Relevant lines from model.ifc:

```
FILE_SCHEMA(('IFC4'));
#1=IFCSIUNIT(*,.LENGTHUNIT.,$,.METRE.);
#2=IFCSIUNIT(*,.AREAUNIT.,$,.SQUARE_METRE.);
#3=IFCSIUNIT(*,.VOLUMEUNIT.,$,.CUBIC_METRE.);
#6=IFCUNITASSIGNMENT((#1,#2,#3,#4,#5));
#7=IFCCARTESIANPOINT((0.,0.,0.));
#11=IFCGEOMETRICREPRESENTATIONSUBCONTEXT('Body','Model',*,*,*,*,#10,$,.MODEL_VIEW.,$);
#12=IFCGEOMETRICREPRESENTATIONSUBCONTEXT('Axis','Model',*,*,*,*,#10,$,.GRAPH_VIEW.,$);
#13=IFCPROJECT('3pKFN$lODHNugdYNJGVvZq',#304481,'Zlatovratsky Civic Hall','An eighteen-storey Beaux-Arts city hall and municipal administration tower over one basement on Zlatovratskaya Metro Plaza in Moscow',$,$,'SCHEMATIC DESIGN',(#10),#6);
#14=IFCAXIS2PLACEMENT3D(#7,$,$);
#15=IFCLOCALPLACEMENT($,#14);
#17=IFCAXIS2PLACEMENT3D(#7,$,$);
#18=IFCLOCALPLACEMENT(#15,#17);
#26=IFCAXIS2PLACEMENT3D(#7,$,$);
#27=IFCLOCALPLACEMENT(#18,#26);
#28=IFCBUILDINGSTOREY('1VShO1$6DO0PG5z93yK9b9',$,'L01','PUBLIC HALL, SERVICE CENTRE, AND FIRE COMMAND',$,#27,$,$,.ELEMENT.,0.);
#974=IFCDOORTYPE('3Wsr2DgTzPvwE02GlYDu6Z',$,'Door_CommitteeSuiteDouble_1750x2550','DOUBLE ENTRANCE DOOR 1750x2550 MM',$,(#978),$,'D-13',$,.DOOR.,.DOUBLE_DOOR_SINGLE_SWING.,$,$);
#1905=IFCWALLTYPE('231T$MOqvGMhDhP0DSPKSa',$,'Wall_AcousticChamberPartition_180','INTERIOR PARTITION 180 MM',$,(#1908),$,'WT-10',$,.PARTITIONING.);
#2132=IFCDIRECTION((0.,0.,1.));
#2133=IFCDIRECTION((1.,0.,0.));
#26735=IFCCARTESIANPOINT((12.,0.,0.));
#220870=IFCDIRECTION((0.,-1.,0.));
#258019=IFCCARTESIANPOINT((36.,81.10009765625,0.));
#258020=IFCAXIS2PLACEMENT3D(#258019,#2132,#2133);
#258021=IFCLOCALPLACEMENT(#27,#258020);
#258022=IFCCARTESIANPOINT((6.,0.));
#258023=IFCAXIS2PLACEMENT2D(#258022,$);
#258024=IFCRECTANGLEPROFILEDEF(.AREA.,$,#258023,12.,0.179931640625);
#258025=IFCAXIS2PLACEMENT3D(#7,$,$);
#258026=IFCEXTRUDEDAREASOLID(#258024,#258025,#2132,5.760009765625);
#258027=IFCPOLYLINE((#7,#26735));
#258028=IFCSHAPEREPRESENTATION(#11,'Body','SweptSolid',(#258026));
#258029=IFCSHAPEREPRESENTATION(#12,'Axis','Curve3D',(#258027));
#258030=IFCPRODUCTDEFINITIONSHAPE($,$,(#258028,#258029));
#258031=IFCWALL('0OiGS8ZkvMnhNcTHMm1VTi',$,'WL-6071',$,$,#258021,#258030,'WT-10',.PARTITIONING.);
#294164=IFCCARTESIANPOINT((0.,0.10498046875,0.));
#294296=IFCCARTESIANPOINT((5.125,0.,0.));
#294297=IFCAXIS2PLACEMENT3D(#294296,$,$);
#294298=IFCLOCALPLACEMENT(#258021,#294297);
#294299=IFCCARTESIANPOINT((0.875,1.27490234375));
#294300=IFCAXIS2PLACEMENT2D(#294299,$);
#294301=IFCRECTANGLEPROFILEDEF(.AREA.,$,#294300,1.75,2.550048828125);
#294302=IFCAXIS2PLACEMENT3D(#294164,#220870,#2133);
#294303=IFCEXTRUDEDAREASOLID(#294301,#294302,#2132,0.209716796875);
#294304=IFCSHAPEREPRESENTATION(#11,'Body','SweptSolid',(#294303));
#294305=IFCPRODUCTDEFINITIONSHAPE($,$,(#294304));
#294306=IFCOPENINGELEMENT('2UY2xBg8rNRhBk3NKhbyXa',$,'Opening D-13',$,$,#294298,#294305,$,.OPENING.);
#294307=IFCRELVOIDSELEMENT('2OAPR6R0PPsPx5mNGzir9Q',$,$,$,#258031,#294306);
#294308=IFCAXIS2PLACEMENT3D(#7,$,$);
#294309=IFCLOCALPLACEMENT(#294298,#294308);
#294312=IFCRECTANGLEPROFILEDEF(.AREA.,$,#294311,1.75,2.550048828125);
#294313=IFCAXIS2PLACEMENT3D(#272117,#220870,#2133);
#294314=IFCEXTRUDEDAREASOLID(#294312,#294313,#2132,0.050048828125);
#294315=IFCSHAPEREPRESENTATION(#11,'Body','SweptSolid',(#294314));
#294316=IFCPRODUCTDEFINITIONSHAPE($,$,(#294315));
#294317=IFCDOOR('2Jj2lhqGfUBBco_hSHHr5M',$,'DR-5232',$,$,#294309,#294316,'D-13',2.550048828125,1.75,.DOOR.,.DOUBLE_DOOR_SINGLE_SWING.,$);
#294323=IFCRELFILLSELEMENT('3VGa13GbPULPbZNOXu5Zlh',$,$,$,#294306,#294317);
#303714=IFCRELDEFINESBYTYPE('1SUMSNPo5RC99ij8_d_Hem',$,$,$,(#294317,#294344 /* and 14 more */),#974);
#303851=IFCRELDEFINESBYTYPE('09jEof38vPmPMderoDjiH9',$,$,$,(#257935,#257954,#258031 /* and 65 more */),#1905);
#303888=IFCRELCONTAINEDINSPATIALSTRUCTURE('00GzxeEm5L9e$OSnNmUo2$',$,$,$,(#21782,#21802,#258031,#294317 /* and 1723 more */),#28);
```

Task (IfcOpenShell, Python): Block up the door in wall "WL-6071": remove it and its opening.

```python
import ifcopenshell
import ifcopenshell.api.feature
import ifcopenshell.api.root
import ifcopenshell.geom
import ifcopenshell.util.shape

model = ifcopenshell.open("model.ifc")
settings = ifcopenshell.geom.settings()


def volume(element):
    """Net volume in cubic metres, openings subtracted."""
    shape = ifcopenshell.geom.create_shape(settings, element)
    return ifcopenshell.util.shape.get_volume(shape.geometry)


door = model.by_id(294317)
opening = door.FillsVoids[0].RelatingOpeningElement
wall = opening.VoidsElements[0].RelatingBuildingElement
before = volume(wall)

ifcopenshell.api.root.remove_product(model, product=door)
ifcopenshell.api.feature.remove_feature(model, feature=opening)

after = volume(wall)

print(f"wall volume {before:.3f} -> {after:.3f} m3")

model.write("model_v2.ifc")
```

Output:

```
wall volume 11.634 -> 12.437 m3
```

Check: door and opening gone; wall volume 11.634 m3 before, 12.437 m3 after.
